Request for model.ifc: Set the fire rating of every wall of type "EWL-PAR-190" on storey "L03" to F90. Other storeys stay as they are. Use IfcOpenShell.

First a look at what the model holds.

```python
import ifcopenshell
import ifcopenshell.util.element

model = ifcopenshell.open("model.ifc")
print(model.schema)
storey = next(s for s in model.by_type("IfcBuildingStorey") if s.Name == "L03")
walls = [e for e in ifcopenshell.util.element.get_decomposition(storey) if e.is_a("IfcWall")]
seen = {}
for e in walls:
    element_type = ifcopenshell.util.element.get_type(e)
    key = (element_type.Name if element_type != e and element_type else None, ifcopenshell.util.element.get_pset(e, "Pset_WallCommon", "FireRating"))
    seen[key] = seen.get(key, 0) + 1
for (name, value), count in sorted(seen.items(), key=str):
    print(count, "x", name, "|", value)
```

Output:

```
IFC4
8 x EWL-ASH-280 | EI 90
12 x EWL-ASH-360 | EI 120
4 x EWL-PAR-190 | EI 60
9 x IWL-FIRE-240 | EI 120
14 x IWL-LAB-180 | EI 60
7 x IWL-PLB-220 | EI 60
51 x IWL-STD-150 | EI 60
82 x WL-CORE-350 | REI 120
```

```python
import ifcopenshell
import ifcopenshell.api.pset
import ifcopenshell.util.element

model = ifcopenshell.open("model.ifc")

storey = next(s for s in model.by_type("IfcBuildingStorey") if s.Name == "L03")
walls = [e for e in ifcopenshell.util.element.get_decomposition(storey) if e.is_a("IfcWall")]

count = 0
for e in walls:
    element_type = ifcopenshell.util.element.get_type(e)
    if element_type in (None, e) or element_type.Name != "EWL-PAR-190":
        continue
    # add_pset returns the element's existing set when there is one.
    pset = ifcopenshell.api.pset.add_pset(model, product=e, name="Pset_WallCommon")
    ifcopenshell.api.pset.edit_pset(model, pset=pset, properties={"FireRating": "F90"})
    count += 1

print(count, "walls updated")

model.write("model_edited.ifc")
```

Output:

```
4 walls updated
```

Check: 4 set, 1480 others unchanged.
